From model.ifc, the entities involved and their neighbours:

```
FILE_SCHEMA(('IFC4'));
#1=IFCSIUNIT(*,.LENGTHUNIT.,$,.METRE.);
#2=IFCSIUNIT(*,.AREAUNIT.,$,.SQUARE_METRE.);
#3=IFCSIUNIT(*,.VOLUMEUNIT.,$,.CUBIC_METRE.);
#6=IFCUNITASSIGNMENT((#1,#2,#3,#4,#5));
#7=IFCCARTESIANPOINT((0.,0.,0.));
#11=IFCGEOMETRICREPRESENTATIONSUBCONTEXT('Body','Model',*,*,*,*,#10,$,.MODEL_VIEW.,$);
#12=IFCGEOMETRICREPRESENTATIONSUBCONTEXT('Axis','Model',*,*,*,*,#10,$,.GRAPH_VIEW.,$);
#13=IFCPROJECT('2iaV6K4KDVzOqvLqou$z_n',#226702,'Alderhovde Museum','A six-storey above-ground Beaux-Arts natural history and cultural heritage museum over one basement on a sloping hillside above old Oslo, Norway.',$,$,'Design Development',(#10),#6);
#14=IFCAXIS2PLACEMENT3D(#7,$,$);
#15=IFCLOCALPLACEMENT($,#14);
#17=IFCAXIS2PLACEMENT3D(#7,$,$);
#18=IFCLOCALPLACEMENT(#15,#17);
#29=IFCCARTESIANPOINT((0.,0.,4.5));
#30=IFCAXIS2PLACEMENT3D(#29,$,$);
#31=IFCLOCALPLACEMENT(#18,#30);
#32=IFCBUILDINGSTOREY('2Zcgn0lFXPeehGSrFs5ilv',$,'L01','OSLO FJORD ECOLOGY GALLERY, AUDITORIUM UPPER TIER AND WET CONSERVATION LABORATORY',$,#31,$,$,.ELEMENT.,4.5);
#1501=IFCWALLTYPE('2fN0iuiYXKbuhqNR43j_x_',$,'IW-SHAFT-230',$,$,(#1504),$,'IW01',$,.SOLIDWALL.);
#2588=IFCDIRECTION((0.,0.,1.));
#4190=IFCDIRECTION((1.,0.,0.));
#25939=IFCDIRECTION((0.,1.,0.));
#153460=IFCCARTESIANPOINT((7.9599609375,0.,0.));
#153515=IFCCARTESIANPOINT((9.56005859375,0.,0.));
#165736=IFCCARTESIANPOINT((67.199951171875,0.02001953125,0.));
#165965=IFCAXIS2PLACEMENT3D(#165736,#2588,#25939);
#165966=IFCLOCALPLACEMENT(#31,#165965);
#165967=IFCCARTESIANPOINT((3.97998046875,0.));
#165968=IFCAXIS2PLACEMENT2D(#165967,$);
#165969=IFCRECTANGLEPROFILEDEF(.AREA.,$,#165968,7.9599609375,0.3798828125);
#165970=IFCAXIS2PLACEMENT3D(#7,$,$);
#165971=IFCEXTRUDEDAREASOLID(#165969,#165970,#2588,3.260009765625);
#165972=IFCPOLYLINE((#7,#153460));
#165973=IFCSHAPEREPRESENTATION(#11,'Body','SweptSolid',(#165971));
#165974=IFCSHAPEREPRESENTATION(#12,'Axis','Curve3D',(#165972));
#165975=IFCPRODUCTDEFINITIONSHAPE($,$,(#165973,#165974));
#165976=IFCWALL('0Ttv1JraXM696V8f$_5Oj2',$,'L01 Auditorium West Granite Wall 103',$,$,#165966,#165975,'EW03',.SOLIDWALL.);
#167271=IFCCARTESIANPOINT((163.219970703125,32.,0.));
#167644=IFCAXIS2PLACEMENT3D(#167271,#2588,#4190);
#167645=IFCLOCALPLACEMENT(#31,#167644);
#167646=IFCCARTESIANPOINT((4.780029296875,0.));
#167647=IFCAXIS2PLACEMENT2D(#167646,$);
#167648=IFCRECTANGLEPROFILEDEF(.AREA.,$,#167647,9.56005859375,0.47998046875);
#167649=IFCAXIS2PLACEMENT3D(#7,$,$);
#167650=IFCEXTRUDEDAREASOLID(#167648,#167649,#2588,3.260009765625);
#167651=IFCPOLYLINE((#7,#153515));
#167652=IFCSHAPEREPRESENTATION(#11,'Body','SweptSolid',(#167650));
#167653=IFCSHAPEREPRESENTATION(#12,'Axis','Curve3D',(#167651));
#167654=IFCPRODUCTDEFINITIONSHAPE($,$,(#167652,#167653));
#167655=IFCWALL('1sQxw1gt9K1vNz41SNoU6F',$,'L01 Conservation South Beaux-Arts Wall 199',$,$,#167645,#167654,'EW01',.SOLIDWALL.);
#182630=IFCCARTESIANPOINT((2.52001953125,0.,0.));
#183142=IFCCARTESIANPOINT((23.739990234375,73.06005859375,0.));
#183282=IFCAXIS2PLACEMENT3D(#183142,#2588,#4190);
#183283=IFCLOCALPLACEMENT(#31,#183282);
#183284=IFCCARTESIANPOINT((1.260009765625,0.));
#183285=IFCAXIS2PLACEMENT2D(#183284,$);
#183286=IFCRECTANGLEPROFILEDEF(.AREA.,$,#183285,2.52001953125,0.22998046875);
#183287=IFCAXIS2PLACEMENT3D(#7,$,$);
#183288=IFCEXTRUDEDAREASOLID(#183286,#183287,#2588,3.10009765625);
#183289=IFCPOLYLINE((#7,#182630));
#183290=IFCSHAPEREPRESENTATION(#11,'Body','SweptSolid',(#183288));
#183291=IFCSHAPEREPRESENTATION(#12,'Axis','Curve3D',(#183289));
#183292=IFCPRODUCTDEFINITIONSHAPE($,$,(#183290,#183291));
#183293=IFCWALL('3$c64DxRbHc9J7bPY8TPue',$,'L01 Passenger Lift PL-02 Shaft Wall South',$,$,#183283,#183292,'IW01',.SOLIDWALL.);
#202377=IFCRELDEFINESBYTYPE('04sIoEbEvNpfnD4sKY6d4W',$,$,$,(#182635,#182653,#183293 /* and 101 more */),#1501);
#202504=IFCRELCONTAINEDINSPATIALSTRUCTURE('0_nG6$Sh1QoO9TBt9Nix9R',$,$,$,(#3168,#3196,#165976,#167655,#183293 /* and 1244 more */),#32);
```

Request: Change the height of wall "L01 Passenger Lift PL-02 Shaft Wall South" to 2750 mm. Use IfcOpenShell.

```python
import ifcopenshell
import ifcopenshell.geom
import ifcopenshell.util.representation
import ifcopenshell.util.shape
import ifcopenshell.util.unit

model = ifcopenshell.open("model.ifc")
unit_scale = ifcopenshell.util.unit.calculate_unit_scale(model)
settings = ifcopenshell.geom.settings()


def volume(element):
    """Net volume in cubic metres, openings subtracted."""
    shape = ifcopenshell.geom.create_shape(settings, element)
    return ifcopenshell.util.shape.get_volume(shape.geometry)


wall = model.by_guid("3$c64DxRbHc9J7bPY8TPue")
before = volume(wall)

body = ifcopenshell.util.representation.get_representation(wall, "Model", "Body")
solid = body.Items[0]
old_height = solid.Depth
solid.Depth = 2.75 / unit_scale
after = volume(wall)

print(f"height {old_height:g} -> {solid.Depth:g}, volume {before:.3f} -> {after:.3f} m3")

model.write("model_updated.ifc")
```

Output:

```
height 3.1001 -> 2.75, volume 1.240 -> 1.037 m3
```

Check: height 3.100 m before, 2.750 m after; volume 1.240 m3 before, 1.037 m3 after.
